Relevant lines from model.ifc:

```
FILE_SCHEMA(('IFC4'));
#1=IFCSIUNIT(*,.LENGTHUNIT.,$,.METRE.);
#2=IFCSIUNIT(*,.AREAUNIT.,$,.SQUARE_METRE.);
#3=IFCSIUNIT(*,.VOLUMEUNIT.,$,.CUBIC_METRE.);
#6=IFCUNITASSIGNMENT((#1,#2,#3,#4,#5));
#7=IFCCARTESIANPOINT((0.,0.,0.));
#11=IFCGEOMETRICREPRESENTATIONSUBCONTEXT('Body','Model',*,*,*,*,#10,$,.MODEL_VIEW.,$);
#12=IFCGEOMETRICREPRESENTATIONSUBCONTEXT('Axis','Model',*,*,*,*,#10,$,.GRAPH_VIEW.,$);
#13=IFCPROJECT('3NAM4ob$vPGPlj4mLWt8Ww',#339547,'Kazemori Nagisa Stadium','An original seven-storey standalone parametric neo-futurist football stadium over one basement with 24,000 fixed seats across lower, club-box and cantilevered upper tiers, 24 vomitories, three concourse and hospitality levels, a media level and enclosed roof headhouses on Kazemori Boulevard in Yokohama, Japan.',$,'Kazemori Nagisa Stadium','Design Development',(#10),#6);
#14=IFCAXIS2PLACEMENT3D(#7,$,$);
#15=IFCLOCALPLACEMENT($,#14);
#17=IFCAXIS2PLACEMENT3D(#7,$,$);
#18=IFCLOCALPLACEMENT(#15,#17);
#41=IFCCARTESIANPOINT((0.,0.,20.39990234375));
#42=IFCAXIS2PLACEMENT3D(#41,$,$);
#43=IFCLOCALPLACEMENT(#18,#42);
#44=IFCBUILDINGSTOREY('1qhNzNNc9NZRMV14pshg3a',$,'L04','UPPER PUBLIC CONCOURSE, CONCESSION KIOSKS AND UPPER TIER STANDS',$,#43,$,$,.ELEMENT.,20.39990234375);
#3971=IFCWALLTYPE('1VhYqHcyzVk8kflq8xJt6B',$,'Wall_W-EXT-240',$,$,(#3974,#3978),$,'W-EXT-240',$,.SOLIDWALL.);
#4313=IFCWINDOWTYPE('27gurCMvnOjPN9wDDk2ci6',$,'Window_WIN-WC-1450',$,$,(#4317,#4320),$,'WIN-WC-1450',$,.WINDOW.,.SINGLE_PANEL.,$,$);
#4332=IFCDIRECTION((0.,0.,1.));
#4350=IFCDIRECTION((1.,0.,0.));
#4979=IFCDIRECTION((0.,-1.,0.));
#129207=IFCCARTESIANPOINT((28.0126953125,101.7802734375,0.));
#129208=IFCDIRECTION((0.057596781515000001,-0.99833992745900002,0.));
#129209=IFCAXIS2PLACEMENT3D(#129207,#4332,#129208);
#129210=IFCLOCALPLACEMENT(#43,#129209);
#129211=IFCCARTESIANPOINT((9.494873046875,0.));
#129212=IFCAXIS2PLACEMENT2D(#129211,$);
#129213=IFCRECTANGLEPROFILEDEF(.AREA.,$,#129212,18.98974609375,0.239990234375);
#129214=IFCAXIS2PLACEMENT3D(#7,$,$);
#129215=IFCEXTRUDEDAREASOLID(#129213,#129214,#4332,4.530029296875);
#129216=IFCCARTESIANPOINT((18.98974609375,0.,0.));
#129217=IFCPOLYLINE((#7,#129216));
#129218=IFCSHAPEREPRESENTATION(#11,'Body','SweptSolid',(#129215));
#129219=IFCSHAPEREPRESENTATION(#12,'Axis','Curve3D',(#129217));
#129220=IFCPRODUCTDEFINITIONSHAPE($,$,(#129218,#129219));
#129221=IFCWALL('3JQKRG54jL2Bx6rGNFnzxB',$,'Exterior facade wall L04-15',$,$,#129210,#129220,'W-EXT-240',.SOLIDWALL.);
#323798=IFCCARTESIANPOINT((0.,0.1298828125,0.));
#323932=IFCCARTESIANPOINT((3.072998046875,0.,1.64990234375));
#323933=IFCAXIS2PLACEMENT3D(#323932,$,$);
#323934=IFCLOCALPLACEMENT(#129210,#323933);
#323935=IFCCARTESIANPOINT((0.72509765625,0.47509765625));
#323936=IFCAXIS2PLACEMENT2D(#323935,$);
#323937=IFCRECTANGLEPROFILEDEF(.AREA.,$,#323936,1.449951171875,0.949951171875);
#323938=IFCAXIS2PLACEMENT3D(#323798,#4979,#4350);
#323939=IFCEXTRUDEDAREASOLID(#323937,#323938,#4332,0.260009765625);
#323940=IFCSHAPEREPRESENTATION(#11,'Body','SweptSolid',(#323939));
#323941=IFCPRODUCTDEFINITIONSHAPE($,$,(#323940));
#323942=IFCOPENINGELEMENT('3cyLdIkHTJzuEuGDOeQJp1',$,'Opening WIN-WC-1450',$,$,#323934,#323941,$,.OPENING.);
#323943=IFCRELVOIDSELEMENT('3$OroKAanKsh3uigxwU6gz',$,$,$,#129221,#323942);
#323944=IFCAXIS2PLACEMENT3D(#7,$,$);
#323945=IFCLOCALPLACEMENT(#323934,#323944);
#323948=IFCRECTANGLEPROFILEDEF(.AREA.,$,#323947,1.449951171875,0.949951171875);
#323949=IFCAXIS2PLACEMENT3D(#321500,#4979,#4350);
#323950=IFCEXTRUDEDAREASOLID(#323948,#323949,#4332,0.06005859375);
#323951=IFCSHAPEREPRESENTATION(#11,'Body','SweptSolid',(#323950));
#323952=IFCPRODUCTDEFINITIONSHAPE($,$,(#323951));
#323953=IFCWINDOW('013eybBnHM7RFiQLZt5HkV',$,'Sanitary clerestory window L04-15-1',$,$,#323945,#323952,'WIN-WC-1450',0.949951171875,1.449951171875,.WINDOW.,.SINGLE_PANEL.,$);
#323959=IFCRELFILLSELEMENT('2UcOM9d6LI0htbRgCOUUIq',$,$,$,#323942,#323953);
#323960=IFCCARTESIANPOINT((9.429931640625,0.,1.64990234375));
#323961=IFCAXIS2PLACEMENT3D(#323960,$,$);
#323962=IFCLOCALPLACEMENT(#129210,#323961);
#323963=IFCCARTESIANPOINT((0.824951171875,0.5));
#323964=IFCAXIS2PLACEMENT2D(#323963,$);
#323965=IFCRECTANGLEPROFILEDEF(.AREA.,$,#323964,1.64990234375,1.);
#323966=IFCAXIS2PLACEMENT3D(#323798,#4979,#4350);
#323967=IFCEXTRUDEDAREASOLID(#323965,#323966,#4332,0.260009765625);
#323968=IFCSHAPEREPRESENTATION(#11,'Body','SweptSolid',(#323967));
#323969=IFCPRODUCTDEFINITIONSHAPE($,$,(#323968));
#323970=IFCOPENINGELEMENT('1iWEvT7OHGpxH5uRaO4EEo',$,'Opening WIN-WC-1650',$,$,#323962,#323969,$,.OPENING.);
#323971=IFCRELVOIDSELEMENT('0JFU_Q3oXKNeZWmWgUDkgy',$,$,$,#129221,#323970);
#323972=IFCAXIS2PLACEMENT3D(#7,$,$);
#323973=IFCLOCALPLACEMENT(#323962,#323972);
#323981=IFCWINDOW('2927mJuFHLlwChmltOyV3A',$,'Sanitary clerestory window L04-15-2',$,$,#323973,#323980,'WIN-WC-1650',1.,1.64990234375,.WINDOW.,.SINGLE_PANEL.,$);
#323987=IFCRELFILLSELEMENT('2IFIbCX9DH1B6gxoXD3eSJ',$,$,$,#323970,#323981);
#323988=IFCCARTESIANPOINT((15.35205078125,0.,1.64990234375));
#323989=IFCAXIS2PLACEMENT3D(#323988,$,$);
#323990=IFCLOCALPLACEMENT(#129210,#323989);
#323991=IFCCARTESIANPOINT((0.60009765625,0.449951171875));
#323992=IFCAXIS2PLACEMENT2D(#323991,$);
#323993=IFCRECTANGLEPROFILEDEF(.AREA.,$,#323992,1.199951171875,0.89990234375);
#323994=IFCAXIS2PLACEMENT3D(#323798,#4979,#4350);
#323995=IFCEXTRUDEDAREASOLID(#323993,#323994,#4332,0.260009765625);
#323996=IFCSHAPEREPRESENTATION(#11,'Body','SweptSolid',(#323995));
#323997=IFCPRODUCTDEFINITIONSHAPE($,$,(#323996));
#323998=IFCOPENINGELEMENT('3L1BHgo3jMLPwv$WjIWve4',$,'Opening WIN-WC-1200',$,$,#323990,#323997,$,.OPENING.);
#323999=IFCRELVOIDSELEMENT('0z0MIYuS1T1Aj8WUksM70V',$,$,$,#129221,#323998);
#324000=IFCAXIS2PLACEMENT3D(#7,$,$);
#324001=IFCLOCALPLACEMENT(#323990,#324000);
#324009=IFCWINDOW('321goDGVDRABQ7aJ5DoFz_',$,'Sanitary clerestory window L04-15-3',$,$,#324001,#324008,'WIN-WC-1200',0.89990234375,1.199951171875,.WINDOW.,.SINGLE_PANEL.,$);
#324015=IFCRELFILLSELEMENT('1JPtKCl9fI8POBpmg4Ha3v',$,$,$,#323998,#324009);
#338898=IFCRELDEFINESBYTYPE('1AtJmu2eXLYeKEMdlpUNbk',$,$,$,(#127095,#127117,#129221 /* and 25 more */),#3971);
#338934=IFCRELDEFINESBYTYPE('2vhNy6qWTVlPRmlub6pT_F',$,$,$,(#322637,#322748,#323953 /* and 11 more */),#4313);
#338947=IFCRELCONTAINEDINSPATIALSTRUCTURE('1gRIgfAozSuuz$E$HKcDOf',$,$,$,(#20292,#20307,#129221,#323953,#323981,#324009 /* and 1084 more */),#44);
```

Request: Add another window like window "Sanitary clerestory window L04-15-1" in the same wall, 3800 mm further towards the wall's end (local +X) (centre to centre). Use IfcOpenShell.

```python
import ifcopenshell
import ifcopenshell.api.feature
import ifcopenshell.api.geometry
import ifcopenshell.api.root
import ifcopenshell.geom
import ifcopenshell.util.element
import ifcopenshell.util.placement
import ifcopenshell.util.shape
import ifcopenshell.util.unit

model = ifcopenshell.open("model.ifc")
unit_scale = ifcopenshell.util.unit.calculate_unit_scale(model)
settings = ifcopenshell.geom.settings()


def volume(element):
    """Net volume in cubic metres, openings subtracted."""
    shape = ifcopenshell.geom.create_shape(settings, element)
    return ifcopenshell.util.shape.get_volume(shape.geometry)


window = model.by_guid("013eybBnHM7RFiQLZt5HkV")
opening = window.FillsVoids[0].RelatingOpeningElement
wall = opening.VoidsElements[0].RelatingBuildingElement
before = volume(wall)
shift = ifcopenshell.util.placement.get_local_placement(wall.ObjectPlacement)[:3, 0] * 3.8 / unit_scale

# copy_class copies the void relationship, type, container and properties, but no geometry.
new_opening = ifcopenshell.api.root.copy_class(model, product=opening)
new_opening.Representation = ifcopenshell.util.element.copy_deep(
    model, opening.Representation, exclude=["IfcGeometricRepresentationContext", "IfcRepresentationMap"]
)
new_window = ifcopenshell.api.root.copy_class(model, product=window)
new_window.Representation = ifcopenshell.util.element.copy_deep(
    model, window.Representation, exclude=["IfcGeometricRepresentationContext", "IfcRepresentationMap"]
)
new_window.Tag = None
ifcopenshell.api.feature.add_filling(model, opening=new_opening, element=new_window)

for old, new in ((opening, new_opening), (window, new_window)):
    matrix = ifcopenshell.util.placement.get_local_placement(old.ObjectPlacement)
    matrix[:3, 3] += shift
    ifcopenshell.api.geometry.edit_object_placement(model, product=new, matrix=matrix, is_si=False)

after = volume(wall)

print(f"wall volume {before:.3f} -> {after:.3f} m3")

model.write("model_updated.ifc")
```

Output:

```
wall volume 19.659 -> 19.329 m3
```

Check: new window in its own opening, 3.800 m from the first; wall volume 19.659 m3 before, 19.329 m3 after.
